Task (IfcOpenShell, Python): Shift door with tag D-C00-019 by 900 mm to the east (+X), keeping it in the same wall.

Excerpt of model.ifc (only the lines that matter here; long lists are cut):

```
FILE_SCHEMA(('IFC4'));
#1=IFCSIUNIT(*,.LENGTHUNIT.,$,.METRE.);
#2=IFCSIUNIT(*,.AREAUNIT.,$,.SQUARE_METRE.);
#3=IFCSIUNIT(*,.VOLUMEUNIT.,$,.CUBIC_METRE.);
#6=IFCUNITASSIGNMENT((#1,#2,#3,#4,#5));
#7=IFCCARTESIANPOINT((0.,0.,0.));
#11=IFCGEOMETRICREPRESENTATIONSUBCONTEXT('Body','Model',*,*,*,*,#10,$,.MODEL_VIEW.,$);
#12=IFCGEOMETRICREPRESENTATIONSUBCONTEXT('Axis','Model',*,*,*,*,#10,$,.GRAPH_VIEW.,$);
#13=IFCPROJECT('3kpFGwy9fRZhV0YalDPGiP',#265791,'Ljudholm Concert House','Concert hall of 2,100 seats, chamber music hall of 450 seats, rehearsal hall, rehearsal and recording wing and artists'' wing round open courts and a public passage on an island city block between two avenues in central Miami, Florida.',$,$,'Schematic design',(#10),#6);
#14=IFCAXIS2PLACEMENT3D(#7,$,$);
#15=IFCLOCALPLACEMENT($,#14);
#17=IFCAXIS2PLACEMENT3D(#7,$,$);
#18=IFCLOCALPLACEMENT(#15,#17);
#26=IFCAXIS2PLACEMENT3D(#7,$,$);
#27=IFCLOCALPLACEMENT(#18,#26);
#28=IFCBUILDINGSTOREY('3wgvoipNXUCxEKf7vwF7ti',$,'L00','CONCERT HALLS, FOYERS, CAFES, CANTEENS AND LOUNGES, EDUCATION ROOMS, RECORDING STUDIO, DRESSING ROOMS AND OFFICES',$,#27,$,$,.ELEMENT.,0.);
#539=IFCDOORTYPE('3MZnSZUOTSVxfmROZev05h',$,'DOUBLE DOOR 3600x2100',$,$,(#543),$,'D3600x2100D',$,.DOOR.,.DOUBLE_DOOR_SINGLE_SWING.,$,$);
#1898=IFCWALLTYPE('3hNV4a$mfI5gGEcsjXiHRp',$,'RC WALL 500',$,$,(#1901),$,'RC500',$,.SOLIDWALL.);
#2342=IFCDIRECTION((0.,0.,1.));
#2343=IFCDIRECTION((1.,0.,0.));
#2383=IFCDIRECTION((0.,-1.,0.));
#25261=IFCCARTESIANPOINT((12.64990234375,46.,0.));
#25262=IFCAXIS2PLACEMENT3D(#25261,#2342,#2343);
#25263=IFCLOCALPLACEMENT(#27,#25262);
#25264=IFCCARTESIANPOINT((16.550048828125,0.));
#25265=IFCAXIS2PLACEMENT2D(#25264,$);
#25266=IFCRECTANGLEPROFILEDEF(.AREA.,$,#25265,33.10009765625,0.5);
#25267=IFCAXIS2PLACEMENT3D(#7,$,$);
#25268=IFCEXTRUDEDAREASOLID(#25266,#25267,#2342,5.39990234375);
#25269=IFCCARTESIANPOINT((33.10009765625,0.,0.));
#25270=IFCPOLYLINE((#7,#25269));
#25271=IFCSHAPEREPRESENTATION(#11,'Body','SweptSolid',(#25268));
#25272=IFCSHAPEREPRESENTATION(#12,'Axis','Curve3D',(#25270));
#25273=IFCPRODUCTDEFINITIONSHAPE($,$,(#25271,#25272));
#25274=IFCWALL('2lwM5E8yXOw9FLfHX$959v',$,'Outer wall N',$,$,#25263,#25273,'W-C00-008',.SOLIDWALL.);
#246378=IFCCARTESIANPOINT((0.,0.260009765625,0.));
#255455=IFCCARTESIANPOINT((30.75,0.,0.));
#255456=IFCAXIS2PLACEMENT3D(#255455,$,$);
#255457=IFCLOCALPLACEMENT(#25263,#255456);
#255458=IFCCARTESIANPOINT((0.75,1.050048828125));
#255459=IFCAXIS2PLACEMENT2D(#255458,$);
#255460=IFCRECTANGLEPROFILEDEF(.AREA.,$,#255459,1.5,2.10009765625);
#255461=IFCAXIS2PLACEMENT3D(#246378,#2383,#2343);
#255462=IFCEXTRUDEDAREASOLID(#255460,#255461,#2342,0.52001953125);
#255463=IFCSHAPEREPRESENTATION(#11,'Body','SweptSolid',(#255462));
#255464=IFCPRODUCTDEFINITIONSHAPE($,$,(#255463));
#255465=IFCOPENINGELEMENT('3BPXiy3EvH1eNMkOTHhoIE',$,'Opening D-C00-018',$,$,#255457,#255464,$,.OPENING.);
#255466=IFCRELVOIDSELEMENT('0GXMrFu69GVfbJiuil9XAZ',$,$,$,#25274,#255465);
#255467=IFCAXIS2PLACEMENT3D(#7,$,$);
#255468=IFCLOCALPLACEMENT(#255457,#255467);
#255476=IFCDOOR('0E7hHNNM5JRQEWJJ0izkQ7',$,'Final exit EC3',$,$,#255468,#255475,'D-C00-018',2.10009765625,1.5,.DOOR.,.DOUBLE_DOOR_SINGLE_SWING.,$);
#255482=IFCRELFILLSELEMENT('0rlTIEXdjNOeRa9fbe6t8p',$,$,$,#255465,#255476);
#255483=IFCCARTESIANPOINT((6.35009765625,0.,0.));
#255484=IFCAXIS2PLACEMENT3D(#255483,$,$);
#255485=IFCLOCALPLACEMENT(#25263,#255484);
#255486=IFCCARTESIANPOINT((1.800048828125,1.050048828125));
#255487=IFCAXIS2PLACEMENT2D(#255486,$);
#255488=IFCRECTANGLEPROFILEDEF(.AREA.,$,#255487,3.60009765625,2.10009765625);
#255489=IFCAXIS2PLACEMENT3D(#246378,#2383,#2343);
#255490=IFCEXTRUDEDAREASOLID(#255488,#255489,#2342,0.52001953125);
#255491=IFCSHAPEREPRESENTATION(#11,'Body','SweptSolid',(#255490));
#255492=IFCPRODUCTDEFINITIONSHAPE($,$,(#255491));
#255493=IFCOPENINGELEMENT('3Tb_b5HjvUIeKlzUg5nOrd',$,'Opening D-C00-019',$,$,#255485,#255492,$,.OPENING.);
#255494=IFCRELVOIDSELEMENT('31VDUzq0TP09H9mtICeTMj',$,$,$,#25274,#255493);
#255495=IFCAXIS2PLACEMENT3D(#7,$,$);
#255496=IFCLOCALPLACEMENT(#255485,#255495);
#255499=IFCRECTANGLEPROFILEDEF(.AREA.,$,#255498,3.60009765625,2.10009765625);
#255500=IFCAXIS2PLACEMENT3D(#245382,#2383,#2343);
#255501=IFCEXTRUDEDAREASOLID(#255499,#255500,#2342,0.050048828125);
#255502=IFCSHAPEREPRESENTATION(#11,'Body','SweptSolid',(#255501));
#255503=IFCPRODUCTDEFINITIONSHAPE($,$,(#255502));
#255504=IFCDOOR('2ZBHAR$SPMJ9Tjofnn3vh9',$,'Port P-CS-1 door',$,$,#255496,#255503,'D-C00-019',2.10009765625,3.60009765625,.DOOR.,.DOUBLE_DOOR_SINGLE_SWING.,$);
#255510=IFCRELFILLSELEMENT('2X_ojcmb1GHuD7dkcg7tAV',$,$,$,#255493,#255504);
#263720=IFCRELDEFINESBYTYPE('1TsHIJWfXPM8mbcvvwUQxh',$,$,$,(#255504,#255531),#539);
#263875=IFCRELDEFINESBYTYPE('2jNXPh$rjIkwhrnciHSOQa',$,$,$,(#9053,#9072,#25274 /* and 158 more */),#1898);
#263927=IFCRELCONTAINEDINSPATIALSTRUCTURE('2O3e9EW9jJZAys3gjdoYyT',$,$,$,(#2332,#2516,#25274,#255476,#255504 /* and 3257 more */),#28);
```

```python
import ifcopenshell
import ifcopenshell.api.geometry
import ifcopenshell.util.placement
import ifcopenshell.util.unit

model = ifcopenshell.open("model.ifc")
unit_scale = ifcopenshell.util.unit.calculate_unit_scale(model)

door = model.by_id(255504)
opening = door.FillsVoids[0].RelatingOpeningElement
wall = opening.VoidsElements[0].RelatingBuildingElement

wall_matrix = ifcopenshell.util.placement.get_local_placement(wall.ObjectPlacement)
shift = wall_matrix[:3, 0] * 0.9 / unit_scale
before = ifcopenshell.util.placement.get_local_placement(door.ObjectPlacement)[:3, 3].copy()

# The door is placed relative to its opening, so it follows when the opening moves.
matrix = ifcopenshell.util.placement.get_local_placement(opening.ObjectPlacement)
matrix[:3, 3] += shift
ifcopenshell.api.geometry.edit_object_placement(
    model, product=opening, matrix=matrix, is_si=False, should_transform_children=True
)

after = ifcopenshell.util.placement.get_local_placement(door.ObjectPlacement)[:3, 3]
print("door moved by", (after - before).round(3) + 0.0)

model.write("model_updated.ifc")
```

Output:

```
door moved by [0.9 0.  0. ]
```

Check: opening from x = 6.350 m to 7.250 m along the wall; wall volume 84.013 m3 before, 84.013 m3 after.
